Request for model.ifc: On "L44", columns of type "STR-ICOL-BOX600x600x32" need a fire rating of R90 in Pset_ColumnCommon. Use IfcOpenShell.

First a look at what the model holds.

```python
import ifcopenshell
import ifcopenshell.util.element

model = ifcopenshell.open("model.ifc")
print(model.schema)
storey = next(s for s in model.by_type("IfcBuildingStorey") if s.Name == "L44")
columns = [e for e in ifcopenshell.util.element.get_decomposition(storey) if e.is_a("IfcColumn")]
seen = {}
for e in columns:
    element_type = ifcopenshell.util.element.get_type(e)
    key = (element_type.Name if element_type != e and element_type else None, ifcopenshell.util.element.get_pset(e, "Pset_ColumnCommon", "FireRating"))
    seen[key] = seen.get(key, 0) + 1
for (name, value), count in sorted(seen.items(), key=str):
    print(count, "x", name, "|", value)
```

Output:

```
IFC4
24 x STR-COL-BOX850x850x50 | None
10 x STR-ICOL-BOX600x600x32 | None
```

```python
import ifcopenshell
import ifcopenshell.api.pset
import ifcopenshell.util.element

model = ifcopenshell.open("model.ifc")

storey = next(s for s in model.by_type("IfcBuildingStorey") if s.Name == "L44")
columns = [e for e in ifcopenshell.util.element.get_decomposition(storey) if e.is_a("IfcColumn")]

count = 0
for e in columns:
    element_type = ifcopenshell.util.element.get_type(e)
    if element_type in (None, e) or element_type.Name != "STR-ICOL-BOX600x600x32":
        continue
    found = ifcopenshell.util.element.get_pset(e, "Pset_ColumnCommon", should_inherit=False)
    if found:
        pset = model.by_id(found["id"])
        if len(ifcopenshell.util.element.get_elements_by_pset(pset)) > 1:
            pset = ifcopenshell.api.pset.unshare_pset(model, products=[e], pset=pset)[0]
    else:
        pset = ifcopenshell.api.pset.add_pset(model, product=e, name="Pset_ColumnCommon")
    ifcopenshell.api.pset.edit_pset(model, pset=pset, properties={"FireRating": "R90"})
    count += 1

print(count, "columns updated")

model.write("model_updated.ifc")
```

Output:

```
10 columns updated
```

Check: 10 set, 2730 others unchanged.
